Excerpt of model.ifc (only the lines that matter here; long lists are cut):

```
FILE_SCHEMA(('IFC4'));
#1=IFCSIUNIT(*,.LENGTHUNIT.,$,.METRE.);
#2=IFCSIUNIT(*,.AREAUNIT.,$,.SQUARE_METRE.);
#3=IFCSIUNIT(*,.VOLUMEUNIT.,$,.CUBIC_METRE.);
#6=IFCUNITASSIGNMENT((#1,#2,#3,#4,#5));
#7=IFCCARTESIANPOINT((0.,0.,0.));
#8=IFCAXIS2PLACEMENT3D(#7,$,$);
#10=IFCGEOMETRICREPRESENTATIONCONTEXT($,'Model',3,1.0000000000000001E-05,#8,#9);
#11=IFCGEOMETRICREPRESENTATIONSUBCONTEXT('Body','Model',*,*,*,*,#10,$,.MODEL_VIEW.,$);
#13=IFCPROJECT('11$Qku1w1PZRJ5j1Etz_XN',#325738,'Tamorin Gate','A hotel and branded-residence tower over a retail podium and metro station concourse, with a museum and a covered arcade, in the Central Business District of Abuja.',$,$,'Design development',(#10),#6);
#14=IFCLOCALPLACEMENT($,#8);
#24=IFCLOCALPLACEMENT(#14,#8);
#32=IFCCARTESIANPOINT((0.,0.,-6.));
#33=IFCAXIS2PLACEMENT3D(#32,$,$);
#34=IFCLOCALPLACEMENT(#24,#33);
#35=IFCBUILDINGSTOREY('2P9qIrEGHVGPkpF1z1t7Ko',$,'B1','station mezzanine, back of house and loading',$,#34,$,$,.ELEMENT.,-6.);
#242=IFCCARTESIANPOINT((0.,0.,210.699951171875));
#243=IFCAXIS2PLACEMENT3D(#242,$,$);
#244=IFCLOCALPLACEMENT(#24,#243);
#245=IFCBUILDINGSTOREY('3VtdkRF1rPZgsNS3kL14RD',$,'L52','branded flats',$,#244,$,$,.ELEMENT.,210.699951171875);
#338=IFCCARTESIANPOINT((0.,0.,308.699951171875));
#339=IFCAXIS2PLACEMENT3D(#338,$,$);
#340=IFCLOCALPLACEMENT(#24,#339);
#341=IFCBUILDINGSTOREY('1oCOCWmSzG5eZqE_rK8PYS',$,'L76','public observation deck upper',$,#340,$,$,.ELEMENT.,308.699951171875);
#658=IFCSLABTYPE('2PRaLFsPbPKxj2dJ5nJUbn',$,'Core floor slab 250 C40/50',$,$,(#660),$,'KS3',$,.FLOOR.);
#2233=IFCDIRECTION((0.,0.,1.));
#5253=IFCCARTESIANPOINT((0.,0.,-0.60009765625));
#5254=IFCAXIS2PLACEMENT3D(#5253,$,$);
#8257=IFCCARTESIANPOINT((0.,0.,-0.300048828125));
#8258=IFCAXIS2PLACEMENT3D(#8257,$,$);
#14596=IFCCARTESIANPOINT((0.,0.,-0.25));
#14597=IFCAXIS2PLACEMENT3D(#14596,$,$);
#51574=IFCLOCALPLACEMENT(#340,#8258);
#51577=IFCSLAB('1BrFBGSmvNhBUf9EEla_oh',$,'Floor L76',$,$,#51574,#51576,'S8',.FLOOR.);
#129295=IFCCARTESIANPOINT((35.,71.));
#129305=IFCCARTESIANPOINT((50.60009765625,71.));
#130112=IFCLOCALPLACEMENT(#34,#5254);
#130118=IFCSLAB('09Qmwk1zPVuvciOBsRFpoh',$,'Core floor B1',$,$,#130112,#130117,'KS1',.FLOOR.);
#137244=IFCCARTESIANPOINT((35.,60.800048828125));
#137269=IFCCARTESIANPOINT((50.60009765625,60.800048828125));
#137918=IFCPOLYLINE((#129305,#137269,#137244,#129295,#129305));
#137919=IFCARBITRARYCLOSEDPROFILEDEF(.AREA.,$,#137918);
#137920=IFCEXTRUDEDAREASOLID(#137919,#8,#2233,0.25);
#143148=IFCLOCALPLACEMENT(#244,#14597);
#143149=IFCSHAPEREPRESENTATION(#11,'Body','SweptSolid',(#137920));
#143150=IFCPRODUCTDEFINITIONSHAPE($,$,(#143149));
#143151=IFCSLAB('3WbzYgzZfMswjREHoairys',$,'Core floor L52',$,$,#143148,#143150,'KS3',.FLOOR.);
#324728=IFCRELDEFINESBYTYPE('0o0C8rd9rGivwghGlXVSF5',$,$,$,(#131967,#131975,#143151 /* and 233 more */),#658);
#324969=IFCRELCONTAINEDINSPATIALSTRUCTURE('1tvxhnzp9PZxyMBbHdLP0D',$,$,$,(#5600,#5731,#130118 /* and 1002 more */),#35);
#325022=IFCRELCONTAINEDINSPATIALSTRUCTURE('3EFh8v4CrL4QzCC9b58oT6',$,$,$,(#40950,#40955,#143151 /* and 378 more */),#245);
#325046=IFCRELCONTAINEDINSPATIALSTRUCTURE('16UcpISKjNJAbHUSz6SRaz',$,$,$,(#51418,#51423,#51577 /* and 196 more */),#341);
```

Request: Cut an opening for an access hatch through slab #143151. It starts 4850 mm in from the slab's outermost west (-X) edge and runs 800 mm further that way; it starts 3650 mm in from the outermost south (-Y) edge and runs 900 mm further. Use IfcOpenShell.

```python
import numpy as np
import ifcopenshell
import ifcopenshell.api.feature
import ifcopenshell.api.geometry
import ifcopenshell.api.root
import ifcopenshell.geom
import ifcopenshell.util.placement
import ifcopenshell.util.representation
import ifcopenshell.util.shape
import ifcopenshell.util.unit

model = ifcopenshell.open("model.ifc")
unit_scale = ifcopenshell.util.unit.calculate_unit_scale(model)
settings = ifcopenshell.geom.settings()


def volume(element):
    """Net volume in cubic metres, openings subtracted."""
    shape = ifcopenshell.geom.create_shape(settings, element)
    return ifcopenshell.util.shape.get_volume(shape.geometry)


slab = model.by_guid("3WbzYgzZfMswjREHoairys")
before = volume(slab)

# Extent in the slab's own axes, in metres. The edges named are its -X and -Y sides.
slab_shape = ifcopenshell.geom.create_shape(settings, slab)
vertices = ifcopenshell.util.shape.get_vertices(slab_shape.geometry)
x_min, y_min, bottom = vertices.min(axis=0)
top = vertices[:, 2].max()

opening = ifcopenshell.api.root.create_entity(model, ifc_class="IfcOpeningElement", name="Access hatch opening", predefined_type="OPENING")
context = ifcopenshell.util.representation.get_context(model, "Model", "Body", "MODEL_VIEW")
width, depth = 0.8, 0.9
outline = [(0.0, 0.0), (width, 0.0), (width, depth), (0.0, depth), (0.0, 0.0)]
# Overshoot both faces by 50 mm so the cut is clean.
shape = ifcopenshell.api.geometry.add_slab_representation(
    model, context=context, depth=top - bottom + 0.1, polyline=outline
)
ifcopenshell.api.geometry.assign_representation(model, product=opening, representation=shape)

matrix = ifcopenshell.util.placement.get_local_placement(slab.ObjectPlacement)
matrix[:, 3] = matrix @ np.append(np.array([x_min + 4.85, y_min + 3.65, bottom - 0.05]) / unit_scale, 1.0)
ifcopenshell.api.geometry.edit_object_placement(model, product=opening, matrix=matrix, is_si=False)
ifcopenshell.api.feature.add_feature(model, feature=opening, element=slab)

after = volume(slab)

print(f"slab volume {before:.3f} -> {after:.3f} m3")

model.write("model_edited.ifc")
```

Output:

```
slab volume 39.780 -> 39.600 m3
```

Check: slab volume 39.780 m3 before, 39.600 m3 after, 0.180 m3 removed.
